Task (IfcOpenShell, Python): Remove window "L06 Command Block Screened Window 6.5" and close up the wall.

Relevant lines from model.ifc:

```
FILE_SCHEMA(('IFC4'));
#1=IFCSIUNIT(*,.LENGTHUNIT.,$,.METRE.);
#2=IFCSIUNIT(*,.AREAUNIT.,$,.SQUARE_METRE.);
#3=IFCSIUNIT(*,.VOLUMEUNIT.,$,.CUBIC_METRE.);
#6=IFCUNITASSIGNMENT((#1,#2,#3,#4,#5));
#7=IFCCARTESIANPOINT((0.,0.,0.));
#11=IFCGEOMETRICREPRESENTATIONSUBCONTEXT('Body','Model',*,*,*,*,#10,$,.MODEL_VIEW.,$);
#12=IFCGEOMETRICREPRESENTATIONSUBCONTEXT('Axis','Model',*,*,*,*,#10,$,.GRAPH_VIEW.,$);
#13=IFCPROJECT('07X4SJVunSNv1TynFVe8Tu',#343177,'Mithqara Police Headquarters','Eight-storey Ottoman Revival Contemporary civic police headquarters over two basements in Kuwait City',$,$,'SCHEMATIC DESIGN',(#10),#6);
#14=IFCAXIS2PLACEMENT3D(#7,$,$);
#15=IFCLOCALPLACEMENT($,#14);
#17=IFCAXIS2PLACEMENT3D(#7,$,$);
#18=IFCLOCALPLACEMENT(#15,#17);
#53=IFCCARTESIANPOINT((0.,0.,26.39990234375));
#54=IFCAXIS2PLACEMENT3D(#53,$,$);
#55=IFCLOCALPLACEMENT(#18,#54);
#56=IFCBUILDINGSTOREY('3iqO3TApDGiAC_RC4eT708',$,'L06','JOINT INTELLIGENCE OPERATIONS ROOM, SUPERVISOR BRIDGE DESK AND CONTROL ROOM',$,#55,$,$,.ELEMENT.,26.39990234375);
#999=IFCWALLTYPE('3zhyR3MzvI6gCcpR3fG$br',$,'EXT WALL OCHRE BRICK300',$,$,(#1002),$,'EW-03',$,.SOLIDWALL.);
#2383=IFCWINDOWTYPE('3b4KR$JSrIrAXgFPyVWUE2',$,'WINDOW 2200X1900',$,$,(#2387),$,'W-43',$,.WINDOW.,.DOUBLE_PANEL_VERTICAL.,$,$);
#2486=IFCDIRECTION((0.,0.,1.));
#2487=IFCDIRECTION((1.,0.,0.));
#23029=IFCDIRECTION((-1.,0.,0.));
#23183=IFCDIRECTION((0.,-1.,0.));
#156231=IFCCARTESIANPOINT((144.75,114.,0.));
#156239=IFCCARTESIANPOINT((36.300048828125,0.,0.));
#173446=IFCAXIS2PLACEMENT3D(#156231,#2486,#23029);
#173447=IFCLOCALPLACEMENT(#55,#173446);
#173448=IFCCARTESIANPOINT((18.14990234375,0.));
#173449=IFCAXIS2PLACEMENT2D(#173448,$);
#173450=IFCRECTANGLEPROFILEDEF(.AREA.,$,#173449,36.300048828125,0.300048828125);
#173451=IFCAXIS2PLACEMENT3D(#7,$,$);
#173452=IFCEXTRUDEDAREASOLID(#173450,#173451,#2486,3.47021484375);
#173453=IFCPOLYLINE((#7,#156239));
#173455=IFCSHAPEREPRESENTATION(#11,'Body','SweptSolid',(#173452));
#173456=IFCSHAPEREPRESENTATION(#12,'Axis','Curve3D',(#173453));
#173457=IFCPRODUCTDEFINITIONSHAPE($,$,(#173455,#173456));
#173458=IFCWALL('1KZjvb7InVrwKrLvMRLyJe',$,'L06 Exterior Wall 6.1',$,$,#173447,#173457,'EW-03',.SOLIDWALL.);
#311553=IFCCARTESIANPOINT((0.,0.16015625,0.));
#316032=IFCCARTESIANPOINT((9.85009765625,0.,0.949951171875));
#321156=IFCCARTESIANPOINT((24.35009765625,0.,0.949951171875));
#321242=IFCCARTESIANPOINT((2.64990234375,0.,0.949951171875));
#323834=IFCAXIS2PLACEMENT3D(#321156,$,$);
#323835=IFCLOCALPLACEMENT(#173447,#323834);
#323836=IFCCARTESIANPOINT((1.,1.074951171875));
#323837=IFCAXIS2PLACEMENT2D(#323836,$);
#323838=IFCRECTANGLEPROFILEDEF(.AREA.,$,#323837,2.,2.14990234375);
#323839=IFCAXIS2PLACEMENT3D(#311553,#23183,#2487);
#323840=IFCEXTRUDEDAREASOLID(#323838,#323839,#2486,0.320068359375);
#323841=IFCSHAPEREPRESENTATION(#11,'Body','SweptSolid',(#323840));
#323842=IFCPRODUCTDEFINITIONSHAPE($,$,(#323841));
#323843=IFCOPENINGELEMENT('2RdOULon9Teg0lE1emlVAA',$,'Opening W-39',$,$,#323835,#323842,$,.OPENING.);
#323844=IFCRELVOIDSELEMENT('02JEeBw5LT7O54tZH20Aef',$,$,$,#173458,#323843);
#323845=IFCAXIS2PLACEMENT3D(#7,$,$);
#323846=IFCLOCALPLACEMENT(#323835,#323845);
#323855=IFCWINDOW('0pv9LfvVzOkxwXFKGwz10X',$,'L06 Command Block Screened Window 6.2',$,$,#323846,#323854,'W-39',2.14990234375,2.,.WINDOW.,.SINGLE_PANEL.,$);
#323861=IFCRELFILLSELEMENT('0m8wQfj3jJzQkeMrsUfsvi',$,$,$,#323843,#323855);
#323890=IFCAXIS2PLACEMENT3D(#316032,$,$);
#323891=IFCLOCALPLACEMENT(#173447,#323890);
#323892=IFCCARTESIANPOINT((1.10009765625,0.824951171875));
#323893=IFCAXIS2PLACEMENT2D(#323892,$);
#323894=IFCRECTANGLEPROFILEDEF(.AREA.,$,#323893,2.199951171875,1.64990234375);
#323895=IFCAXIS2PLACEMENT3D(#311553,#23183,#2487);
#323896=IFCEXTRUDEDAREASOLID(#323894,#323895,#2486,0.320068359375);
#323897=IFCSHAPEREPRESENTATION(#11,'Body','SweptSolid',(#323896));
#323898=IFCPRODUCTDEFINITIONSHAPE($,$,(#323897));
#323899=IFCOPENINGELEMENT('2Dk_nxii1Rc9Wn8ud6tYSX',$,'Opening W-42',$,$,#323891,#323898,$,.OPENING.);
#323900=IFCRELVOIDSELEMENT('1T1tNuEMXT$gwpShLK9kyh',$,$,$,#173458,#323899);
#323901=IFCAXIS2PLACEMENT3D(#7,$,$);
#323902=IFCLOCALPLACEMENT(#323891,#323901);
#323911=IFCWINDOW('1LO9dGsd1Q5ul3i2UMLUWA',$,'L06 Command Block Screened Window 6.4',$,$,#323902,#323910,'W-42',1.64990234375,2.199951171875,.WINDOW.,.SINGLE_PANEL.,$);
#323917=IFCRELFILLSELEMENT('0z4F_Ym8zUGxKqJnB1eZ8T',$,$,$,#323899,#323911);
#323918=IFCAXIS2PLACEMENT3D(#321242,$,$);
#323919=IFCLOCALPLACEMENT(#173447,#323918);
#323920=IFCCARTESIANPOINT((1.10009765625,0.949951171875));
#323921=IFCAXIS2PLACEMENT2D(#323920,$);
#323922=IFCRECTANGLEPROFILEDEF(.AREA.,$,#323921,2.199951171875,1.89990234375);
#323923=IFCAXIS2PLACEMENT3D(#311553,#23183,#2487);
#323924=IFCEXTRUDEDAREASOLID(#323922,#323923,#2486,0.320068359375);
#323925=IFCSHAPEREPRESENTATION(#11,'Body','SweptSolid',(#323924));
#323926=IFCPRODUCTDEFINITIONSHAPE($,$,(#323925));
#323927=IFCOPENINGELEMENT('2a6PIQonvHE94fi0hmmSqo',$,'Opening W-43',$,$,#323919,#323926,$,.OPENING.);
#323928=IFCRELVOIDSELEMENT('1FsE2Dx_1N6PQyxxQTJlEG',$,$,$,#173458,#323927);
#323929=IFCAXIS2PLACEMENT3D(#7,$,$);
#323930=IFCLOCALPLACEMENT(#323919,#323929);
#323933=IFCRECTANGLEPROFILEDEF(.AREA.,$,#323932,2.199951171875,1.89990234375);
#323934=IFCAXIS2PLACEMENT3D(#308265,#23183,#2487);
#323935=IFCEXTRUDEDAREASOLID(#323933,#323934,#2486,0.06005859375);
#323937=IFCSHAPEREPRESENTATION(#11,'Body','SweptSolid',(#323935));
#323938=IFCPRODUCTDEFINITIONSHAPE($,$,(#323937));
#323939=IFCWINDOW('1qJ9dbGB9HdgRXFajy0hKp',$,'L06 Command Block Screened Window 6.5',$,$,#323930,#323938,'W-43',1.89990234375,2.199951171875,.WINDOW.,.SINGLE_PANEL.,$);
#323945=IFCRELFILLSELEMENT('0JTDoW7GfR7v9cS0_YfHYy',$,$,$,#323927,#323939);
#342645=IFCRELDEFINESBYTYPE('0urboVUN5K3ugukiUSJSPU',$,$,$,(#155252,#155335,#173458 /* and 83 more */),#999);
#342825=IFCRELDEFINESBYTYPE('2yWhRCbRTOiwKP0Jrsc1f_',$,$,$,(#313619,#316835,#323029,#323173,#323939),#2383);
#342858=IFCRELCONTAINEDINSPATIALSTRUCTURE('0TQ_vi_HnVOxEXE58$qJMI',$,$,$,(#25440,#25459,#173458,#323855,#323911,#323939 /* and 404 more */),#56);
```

```python
import ifcopenshell
import ifcopenshell.api.feature
import ifcopenshell.api.root
import ifcopenshell.geom
import ifcopenshell.util.shape

model = ifcopenshell.open("model.ifc")
settings = ifcopenshell.geom.settings()


def volume(element):
    """Net volume in cubic metres, openings subtracted."""
    shape = ifcopenshell.geom.create_shape(settings, element)
    return ifcopenshell.util.shape.get_volume(shape.geometry)


window = model.by_guid("1qJ9dbGB9HdgRXFajy0hKp")
opening = window.FillsVoids[0].RelatingOpeningElement
wall = opening.VoidsElements[0].RelatingBuildingElement
before = volume(wall)

ifcopenshell.api.root.remove_product(model, product=window)
ifcopenshell.api.feature.remove_feature(model, feature=opening)

after = volume(wall)

print(f"wall volume {before:.3f} -> {after:.3f} m3")

model.write("model_rev.ifc")
```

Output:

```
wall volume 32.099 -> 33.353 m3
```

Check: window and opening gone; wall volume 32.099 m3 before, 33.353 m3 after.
